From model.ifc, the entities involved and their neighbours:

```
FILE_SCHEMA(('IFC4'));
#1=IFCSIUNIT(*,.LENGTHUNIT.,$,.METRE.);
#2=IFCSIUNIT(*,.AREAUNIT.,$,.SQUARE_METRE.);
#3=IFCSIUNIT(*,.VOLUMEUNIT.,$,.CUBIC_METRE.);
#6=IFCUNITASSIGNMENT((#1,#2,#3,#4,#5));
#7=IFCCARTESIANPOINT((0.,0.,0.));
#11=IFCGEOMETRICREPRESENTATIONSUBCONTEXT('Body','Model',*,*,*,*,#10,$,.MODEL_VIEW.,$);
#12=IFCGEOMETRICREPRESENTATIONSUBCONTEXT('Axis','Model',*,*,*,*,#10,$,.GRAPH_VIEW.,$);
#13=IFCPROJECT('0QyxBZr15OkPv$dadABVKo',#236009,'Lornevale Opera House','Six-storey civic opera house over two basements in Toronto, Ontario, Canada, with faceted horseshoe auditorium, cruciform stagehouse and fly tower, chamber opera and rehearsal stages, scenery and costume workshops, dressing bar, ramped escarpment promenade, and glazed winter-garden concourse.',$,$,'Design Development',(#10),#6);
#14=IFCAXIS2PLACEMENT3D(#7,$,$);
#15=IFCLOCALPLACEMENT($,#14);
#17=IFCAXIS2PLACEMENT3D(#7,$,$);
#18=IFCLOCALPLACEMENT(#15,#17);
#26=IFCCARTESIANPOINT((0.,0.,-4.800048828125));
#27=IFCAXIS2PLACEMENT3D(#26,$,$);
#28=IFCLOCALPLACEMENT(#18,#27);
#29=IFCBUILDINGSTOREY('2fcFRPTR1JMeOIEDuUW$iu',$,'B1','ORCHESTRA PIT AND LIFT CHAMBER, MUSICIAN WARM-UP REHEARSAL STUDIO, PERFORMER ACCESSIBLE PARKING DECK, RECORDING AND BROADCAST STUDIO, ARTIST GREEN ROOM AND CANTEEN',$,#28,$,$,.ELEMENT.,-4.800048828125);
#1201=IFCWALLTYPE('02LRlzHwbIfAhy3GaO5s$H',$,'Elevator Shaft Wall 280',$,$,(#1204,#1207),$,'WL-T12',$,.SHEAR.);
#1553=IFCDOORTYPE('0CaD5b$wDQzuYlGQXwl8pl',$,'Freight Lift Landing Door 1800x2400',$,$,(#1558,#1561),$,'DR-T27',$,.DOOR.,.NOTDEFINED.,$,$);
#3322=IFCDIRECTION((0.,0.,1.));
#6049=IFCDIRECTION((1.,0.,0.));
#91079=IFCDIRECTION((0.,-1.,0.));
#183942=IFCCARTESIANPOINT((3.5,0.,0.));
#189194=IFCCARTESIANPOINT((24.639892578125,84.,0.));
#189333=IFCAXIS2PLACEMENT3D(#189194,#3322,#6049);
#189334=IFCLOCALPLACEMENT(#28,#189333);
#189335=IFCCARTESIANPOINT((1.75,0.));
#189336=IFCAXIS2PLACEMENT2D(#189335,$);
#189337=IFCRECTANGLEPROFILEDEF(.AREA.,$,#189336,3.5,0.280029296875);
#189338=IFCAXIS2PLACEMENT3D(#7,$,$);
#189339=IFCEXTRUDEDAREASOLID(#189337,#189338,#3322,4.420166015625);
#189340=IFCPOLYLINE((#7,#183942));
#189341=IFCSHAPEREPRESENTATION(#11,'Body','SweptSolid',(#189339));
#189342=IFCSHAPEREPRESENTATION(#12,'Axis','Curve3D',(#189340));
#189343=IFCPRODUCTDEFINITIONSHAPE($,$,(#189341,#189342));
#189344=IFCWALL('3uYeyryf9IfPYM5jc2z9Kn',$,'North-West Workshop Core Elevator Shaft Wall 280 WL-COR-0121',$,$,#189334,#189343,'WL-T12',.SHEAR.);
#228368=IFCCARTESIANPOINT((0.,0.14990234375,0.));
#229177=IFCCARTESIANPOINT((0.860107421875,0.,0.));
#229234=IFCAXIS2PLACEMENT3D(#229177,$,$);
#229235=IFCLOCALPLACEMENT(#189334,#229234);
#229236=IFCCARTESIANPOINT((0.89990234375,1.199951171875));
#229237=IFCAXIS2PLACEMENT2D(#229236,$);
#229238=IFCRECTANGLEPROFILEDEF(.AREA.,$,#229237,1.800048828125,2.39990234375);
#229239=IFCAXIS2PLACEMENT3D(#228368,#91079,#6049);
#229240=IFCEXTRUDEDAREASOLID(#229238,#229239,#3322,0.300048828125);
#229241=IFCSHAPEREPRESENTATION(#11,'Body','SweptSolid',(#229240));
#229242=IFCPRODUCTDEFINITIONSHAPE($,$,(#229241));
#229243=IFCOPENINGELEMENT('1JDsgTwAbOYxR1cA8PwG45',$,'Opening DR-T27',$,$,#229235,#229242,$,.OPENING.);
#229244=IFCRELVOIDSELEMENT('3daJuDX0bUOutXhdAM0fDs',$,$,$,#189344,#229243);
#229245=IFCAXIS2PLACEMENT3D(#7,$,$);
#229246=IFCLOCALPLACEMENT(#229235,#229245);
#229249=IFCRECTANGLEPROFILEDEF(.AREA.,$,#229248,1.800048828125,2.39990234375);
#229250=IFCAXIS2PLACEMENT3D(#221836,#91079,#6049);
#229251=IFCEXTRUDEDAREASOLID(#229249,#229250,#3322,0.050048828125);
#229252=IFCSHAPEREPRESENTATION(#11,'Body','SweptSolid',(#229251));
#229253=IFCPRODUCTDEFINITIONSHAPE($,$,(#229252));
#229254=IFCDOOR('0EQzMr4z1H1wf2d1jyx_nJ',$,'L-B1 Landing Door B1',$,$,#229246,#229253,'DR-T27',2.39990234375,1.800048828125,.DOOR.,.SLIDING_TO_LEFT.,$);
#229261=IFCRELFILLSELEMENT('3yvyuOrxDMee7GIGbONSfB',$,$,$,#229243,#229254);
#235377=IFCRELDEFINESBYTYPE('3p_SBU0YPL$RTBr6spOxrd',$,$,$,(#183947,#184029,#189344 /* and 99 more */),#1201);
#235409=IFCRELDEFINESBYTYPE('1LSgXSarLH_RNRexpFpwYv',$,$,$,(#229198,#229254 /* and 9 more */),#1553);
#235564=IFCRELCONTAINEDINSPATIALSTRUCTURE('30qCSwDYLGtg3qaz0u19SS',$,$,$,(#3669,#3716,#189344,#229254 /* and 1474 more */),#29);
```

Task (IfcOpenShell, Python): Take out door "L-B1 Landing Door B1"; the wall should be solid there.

```python
import ifcopenshell
import ifcopenshell.api.feature
import ifcopenshell.api.root
import ifcopenshell.geom
import ifcopenshell.util.shape

model = ifcopenshell.open("model.ifc")
settings = ifcopenshell.geom.settings()


def volume(element):
    """Net volume in cubic metres, openings subtracted."""
    shape = ifcopenshell.geom.create_shape(settings, element)
    return ifcopenshell.util.shape.get_volume(shape.geometry)


door = model.by_guid("0EQzMr4z1H1wf2d1jyx_nJ")
opening = door.FillsVoids[0].RelatingOpeningElement
wall = opening.VoidsElements[0].RelatingBuildingElement
before = volume(wall)

ifcopenshell.api.root.remove_product(model, product=door)
ifcopenshell.api.feature.remove_feature(model, feature=opening)

after = volume(wall)

print(f"wall volume {before:.3f} -> {after:.3f} m3")

model.write("model-out.ifc")
```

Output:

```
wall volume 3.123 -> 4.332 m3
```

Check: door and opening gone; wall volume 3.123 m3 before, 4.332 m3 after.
